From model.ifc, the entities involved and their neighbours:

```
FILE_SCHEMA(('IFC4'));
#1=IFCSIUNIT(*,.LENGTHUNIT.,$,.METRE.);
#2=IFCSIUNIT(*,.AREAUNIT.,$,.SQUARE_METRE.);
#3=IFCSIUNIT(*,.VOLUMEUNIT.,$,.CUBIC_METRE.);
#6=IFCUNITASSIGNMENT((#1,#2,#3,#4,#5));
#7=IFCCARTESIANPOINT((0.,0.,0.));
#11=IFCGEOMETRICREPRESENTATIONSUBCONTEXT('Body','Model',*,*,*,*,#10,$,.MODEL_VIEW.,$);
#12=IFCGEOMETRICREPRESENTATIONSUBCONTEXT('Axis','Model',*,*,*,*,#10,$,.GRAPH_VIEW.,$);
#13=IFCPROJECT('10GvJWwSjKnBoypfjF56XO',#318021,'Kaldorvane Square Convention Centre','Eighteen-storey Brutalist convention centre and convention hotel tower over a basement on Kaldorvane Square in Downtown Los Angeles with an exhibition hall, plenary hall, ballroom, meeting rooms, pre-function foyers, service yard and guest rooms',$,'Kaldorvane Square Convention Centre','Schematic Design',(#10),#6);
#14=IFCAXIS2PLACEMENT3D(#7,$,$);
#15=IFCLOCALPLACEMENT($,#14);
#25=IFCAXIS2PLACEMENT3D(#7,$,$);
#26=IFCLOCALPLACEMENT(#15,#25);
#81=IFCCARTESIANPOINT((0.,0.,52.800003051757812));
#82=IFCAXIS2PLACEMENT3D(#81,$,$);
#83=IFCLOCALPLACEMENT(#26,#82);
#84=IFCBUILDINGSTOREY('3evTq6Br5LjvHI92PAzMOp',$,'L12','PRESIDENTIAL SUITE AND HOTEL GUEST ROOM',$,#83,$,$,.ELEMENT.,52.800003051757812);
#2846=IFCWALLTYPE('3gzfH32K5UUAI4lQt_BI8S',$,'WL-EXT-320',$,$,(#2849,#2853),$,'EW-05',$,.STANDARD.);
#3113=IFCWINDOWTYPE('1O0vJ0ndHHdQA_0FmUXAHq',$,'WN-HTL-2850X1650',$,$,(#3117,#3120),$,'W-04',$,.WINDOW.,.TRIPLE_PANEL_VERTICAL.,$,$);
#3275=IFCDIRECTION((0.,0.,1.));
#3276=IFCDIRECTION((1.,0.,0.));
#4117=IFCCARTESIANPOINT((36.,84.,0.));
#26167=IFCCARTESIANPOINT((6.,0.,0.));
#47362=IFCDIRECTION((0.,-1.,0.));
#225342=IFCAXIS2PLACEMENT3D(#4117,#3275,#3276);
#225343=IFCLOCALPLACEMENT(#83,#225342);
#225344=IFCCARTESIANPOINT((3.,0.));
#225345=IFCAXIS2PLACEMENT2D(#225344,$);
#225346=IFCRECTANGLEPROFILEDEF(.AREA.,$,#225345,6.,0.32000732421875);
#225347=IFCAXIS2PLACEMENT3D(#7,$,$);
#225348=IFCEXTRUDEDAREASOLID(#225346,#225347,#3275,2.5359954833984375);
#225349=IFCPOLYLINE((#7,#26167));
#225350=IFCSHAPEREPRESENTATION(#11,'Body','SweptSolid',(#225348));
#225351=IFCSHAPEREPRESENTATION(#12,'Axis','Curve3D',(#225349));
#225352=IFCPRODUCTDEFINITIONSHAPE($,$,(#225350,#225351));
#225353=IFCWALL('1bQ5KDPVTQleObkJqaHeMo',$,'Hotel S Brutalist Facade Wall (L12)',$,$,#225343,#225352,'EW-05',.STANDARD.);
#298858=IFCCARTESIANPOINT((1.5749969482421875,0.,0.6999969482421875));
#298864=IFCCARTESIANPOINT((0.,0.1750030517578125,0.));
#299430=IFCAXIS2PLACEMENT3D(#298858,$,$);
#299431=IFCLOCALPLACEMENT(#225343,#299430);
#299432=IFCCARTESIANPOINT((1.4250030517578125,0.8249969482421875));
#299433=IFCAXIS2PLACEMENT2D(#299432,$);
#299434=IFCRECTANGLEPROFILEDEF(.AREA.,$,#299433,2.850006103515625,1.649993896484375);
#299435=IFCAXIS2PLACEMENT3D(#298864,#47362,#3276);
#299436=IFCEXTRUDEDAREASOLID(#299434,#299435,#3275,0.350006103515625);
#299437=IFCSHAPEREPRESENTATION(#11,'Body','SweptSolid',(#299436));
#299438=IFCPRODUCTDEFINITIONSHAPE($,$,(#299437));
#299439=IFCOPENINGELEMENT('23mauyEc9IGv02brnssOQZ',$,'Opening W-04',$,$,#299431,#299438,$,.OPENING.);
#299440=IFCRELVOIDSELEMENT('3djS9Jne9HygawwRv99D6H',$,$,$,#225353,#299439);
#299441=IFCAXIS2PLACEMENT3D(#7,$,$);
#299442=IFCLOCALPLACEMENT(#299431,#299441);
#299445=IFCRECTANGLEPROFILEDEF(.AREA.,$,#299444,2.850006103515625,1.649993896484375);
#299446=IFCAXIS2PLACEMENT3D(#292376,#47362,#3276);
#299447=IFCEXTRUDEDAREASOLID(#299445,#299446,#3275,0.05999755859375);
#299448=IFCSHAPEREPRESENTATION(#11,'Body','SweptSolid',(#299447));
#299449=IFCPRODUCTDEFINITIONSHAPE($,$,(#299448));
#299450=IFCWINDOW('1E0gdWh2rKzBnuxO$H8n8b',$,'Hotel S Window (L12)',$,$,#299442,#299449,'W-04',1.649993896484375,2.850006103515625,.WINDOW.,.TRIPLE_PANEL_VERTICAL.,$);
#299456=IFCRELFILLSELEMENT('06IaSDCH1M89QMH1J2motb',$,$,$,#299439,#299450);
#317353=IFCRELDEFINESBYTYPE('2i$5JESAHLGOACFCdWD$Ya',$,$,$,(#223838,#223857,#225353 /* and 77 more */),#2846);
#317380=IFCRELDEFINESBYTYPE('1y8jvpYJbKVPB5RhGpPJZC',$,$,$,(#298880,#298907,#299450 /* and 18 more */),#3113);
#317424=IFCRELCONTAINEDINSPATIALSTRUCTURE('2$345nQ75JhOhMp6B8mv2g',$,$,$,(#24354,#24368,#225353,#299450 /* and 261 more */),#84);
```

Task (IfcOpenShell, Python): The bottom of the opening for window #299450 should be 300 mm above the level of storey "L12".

```python
import numpy as np
import ifcopenshell
import ifcopenshell.api.geometry
import ifcopenshell.geom
import ifcopenshell.util.element
import ifcopenshell.util.placement
import ifcopenshell.util.shape
import ifcopenshell.util.unit

model = ifcopenshell.open("model.ifc")
unit_scale = ifcopenshell.util.unit.calculate_unit_scale(model)

window = model.by_id(299450)
opening = window.FillsVoids[0].RelatingOpeningElement
storey = ifcopenshell.util.element.get_container(window, ifc_class="IfcBuildingStorey")
level = ifcopenshell.util.placement.get_local_placement(storey.ObjectPlacement)[2, 3]

# The opening's origin need not be at the sill, so measure its lowest point.
shape = ifcopenshell.geom.create_shape(ifcopenshell.geom.settings(), opening)
bottom = ifcopenshell.util.shape.get_shape_bottom_elevation(shape, shape.geometry) / unit_scale
dz = level + 0.3 / unit_scale - bottom

shift = np.array([0.0, 0.0, dz])
# The window is placed relative to its opening, so it follows when the opening moves.
matrix = ifcopenshell.util.placement.get_local_placement(opening.ObjectPlacement)
matrix[:3, 3] += shift
ifcopenshell.api.geometry.edit_object_placement(
    model, product=opening, matrix=matrix, is_si=False, should_transform_children=True
)

print(f"moved by {dz * unit_scale:+.3f} m")

model.write("model-out.ifc")
```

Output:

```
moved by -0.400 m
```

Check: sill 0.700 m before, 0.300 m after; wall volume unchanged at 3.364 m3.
